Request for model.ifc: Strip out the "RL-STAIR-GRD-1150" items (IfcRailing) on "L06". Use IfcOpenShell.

First a look at what the model holds.

```python
import ifcopenshell
import ifcopenshell.util.element

model = ifcopenshell.open("model.ifc")
print(model.schema)
storey = next(s for s in model.by_type("IfcBuildingStorey") if s.Name == "L06")
railings = [e for e in ifcopenshell.util.element.get_decomposition(storey) if e.is_a("IfcRailing")]
seen = {}
for e in railings:
    element_type = ifcopenshell.util.element.get_type(e)
    name = element_type.Name if element_type not in (None, e) else None
    seen[name] = seen.get(name, 0) + 1
for name, count in sorted(seen.items(), key=str):
    print(count, "x", name)
```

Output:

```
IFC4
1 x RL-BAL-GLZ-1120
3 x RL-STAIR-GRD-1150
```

```python
import ifcopenshell
import ifcopenshell.api.root
import ifcopenshell.util.element

model = ifcopenshell.open("model.ifc")

storey = next(s for s in model.by_type("IfcBuildingStorey") if s.Name == "L06")
railings = [e for e in ifcopenshell.util.element.get_decomposition(storey) if e.is_a("IfcRailing")]
targets = [e for e in railings if (t := ifcopenshell.util.element.get_type(e)) not in (None, e) and t.Name == "RL-STAIR-GRD-1150"]

for e in targets:
    ifcopenshell.api.root.remove_product(model, product=e)
print(len(targets), "removed")

model.write("model_rev.ifc")
```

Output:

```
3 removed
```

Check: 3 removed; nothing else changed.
